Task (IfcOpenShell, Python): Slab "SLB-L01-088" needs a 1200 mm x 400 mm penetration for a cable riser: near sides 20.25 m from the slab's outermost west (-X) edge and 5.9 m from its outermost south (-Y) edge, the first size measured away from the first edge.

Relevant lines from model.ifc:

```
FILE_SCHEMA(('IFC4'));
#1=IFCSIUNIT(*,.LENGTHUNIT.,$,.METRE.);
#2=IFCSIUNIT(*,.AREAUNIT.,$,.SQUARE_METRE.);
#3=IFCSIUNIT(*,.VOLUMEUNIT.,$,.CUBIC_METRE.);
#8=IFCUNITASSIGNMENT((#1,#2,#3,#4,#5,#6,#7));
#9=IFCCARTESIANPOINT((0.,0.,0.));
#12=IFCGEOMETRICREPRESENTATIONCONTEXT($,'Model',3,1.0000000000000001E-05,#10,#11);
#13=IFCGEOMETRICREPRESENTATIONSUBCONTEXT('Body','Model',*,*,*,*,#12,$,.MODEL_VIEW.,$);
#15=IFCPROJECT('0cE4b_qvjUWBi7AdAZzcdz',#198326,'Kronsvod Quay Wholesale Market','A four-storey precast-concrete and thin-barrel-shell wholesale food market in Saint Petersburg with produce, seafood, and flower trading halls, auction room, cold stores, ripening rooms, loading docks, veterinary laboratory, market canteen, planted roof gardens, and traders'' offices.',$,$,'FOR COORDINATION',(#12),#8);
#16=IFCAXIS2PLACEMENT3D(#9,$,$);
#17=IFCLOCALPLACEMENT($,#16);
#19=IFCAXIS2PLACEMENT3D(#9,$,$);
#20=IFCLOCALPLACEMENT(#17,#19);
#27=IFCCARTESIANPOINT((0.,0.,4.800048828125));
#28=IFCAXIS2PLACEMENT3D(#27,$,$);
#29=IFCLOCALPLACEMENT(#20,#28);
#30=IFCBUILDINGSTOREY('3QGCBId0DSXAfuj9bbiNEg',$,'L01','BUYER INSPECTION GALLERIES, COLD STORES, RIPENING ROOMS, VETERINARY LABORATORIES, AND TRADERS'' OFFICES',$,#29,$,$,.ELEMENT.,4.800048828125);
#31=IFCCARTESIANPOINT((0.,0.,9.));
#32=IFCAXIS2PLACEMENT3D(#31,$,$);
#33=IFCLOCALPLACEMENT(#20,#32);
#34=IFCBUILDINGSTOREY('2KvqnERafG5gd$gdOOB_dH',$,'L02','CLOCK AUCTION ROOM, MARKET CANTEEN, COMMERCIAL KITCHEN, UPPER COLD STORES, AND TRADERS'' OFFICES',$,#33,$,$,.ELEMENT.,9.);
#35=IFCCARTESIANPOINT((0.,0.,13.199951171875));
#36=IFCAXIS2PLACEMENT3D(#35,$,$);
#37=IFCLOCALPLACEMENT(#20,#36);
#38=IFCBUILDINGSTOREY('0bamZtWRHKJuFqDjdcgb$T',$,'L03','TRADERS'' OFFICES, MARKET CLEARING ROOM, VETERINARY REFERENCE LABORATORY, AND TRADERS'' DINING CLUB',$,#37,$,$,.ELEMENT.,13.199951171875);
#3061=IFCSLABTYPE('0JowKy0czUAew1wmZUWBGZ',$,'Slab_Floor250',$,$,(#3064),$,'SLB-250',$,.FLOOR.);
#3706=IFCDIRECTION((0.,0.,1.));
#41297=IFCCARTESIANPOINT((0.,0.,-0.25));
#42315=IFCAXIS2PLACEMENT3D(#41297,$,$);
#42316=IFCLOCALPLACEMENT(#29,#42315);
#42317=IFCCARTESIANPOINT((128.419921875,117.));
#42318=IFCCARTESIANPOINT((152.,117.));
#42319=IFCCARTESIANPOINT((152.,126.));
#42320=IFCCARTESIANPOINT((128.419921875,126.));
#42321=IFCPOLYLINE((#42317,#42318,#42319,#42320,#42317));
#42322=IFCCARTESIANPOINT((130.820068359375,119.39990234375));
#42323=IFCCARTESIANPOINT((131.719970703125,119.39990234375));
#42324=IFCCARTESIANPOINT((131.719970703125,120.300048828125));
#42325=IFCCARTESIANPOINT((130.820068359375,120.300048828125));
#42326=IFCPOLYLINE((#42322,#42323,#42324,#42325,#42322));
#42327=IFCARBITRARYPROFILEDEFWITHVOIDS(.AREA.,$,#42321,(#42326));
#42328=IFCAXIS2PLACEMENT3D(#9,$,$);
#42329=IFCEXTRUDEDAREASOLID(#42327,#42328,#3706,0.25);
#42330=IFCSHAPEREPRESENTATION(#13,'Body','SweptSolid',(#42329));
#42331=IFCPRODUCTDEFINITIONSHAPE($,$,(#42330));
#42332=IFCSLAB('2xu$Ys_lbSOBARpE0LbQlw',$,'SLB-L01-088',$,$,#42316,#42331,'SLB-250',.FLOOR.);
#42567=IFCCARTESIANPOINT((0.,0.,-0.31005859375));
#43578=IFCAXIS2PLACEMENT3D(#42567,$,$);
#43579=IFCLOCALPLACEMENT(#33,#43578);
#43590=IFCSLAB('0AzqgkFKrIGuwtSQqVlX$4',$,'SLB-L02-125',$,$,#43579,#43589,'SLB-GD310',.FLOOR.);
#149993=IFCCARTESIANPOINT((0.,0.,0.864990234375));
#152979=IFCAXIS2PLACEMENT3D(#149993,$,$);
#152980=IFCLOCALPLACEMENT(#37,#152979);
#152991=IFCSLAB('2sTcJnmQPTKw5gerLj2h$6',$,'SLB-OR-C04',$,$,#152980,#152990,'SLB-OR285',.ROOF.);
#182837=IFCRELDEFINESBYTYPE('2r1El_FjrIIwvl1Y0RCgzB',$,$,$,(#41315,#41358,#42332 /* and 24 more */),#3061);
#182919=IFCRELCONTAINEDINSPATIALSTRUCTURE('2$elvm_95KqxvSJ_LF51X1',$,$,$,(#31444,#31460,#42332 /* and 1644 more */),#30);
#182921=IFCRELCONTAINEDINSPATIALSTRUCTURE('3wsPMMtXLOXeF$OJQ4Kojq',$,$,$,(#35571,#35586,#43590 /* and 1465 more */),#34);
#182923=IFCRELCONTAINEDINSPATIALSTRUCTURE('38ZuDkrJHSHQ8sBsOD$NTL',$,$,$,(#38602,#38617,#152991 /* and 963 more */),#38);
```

```python
import numpy as np
import ifcopenshell
import ifcopenshell.api.feature
import ifcopenshell.api.geometry
import ifcopenshell.api.root
import ifcopenshell.geom
import ifcopenshell.util.placement
import ifcopenshell.util.representation
import ifcopenshell.util.shape
import ifcopenshell.util.unit

model = ifcopenshell.open("model.ifc")
unit_scale = ifcopenshell.util.unit.calculate_unit_scale(model)
settings = ifcopenshell.geom.settings()


def volume(element):
    """Net volume in cubic metres, openings subtracted."""
    shape = ifcopenshell.geom.create_shape(settings, element)
    return ifcopenshell.util.shape.get_volume(shape.geometry)


slab = model.by_guid("2xu$Ys_lbSOBARpE0LbQlw")
before = volume(slab)

# Extent in the slab's own axes, in metres. The edges named are its -X and -Y sides.
slab_shape = ifcopenshell.geom.create_shape(settings, slab)
vertices = ifcopenshell.util.shape.get_vertices(slab_shape.geometry)
x_min, y_min, bottom = vertices.min(axis=0)
top = vertices[:, 2].max()

opening = ifcopenshell.api.root.create_entity(model, ifc_class="IfcOpeningElement", name="Cable riser opening", predefined_type="OPENING")
context = ifcopenshell.util.representation.get_context(model, "Model", "Body", "MODEL_VIEW")
width, depth = 1.2, 0.4
outline = [(0.0, 0.0), (width, 0.0), (width, depth), (0.0, depth), (0.0, 0.0)]
# Overshoot both faces by 50 mm so the cut is clean.
shape = ifcopenshell.api.geometry.add_slab_representation(
    model, context=context, depth=top - bottom + 0.1, polyline=outline
)
ifcopenshell.api.geometry.assign_representation(model, product=opening, representation=shape)

matrix = ifcopenshell.util.placement.get_local_placement(slab.ObjectPlacement)
matrix[:, 3] = matrix @ np.append(np.array([x_min + 20.25, y_min + 5.9, bottom - 0.05]) / unit_scale, 1.0)
ifcopenshell.api.geometry.edit_object_placement(model, product=opening, matrix=matrix, is_si=False)
ifcopenshell.api.feature.add_feature(model, feature=opening, element=slab)

after = volume(slab)

print(f"slab volume {before:.3f} -> {after:.3f} m3")

model.write("model_v2.ifc")
```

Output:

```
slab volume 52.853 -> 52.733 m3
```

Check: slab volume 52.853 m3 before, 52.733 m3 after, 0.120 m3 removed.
